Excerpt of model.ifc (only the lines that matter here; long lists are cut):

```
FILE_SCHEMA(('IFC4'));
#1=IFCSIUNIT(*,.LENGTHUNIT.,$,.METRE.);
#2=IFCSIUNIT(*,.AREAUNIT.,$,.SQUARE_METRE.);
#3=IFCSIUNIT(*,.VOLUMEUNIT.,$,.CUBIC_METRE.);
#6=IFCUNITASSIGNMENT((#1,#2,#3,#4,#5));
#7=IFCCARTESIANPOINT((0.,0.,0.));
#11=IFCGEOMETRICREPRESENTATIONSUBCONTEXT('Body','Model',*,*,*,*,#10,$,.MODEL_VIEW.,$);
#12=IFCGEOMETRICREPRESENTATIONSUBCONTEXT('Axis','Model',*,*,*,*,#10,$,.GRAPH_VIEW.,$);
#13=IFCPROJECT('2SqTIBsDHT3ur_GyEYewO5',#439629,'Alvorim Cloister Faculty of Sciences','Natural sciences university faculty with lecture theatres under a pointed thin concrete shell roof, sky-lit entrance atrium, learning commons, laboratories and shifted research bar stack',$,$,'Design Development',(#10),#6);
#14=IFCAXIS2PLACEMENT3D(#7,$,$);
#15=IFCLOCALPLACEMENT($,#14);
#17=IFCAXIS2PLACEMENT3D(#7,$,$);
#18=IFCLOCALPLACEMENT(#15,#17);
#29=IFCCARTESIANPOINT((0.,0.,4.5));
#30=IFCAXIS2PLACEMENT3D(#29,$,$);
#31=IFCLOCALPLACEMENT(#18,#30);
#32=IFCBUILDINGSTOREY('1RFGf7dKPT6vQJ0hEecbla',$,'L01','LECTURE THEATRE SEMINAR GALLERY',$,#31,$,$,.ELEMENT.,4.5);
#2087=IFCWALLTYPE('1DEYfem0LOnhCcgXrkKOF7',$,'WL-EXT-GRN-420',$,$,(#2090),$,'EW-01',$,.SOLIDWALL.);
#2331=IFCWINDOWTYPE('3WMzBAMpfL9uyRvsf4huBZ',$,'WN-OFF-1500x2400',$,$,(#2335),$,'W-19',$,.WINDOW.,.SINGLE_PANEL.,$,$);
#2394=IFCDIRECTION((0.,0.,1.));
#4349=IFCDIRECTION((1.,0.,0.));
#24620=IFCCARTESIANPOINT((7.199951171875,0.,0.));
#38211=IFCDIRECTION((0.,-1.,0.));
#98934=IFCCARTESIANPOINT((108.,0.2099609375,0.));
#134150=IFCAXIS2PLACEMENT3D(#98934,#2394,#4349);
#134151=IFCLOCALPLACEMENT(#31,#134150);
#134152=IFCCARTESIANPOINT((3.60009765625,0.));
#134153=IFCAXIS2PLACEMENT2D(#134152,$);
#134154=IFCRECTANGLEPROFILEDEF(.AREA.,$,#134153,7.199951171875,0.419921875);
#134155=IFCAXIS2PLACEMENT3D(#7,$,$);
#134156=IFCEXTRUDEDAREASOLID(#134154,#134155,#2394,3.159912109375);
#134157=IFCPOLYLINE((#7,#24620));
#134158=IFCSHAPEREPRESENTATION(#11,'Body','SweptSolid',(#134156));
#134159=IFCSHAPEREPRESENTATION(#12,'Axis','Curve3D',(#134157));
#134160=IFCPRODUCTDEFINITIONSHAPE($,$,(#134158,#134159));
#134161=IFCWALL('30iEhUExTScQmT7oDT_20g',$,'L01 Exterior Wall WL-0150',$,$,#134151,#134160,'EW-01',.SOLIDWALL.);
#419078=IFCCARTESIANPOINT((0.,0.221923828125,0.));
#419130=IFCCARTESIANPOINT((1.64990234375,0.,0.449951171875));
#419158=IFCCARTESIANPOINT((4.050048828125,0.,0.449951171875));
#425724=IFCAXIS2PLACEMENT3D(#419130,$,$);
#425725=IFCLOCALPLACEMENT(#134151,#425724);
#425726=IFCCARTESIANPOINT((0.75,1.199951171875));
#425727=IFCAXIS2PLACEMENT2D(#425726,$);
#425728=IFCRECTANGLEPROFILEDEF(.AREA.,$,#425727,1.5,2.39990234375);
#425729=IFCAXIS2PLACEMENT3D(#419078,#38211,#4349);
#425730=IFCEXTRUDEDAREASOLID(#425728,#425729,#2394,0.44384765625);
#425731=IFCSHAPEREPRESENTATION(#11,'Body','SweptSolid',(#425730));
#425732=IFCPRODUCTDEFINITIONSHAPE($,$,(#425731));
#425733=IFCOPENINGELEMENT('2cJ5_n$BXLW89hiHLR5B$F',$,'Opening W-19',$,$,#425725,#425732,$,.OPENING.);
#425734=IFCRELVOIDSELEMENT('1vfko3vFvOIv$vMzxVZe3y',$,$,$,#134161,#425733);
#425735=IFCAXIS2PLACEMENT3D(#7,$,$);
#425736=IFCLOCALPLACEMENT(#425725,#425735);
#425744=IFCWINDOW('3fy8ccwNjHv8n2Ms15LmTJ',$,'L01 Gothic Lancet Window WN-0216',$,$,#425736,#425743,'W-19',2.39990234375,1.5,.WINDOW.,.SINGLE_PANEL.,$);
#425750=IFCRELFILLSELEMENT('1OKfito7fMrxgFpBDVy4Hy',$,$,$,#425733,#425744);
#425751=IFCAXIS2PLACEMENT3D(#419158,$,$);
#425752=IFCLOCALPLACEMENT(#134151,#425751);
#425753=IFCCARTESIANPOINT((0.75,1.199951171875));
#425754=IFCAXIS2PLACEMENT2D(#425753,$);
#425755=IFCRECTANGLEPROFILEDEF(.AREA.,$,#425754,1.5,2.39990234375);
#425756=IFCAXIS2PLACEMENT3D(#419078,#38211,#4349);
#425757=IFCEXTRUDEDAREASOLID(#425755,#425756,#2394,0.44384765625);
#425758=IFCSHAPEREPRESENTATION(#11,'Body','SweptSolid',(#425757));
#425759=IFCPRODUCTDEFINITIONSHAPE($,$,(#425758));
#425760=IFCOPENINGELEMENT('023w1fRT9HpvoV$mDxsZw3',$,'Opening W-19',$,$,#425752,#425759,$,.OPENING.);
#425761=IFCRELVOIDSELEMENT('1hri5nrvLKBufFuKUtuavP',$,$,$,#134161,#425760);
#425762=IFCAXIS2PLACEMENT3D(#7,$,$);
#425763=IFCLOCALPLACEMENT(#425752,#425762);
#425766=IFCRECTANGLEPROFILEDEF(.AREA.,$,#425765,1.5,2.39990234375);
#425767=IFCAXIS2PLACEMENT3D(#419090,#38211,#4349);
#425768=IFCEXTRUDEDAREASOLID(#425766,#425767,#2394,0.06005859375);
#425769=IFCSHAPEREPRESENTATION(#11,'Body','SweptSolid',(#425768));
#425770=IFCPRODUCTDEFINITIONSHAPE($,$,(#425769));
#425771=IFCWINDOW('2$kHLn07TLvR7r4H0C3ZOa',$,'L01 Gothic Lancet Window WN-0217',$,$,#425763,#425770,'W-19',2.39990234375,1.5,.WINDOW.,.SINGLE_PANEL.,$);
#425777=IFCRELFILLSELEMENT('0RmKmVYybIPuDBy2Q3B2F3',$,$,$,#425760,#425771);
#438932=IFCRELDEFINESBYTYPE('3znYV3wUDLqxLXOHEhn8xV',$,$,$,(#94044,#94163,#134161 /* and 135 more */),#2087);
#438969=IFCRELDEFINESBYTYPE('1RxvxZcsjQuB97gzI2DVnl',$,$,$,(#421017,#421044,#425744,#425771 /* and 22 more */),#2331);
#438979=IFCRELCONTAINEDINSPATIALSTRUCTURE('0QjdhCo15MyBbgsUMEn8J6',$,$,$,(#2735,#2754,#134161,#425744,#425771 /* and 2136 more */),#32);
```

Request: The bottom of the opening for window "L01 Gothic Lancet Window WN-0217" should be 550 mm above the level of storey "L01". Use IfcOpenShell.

```python
import numpy as np
import ifcopenshell
import ifcopenshell.api.geometry
import ifcopenshell.geom
import ifcopenshell.util.element
import ifcopenshell.util.placement
import ifcopenshell.util.shape
import ifcopenshell.util.unit

model = ifcopenshell.open("model.ifc")
unit_scale = ifcopenshell.util.unit.calculate_unit_scale(model)

window = model.by_id(425771)
opening = window.FillsVoids[0].RelatingOpeningElement
storey = ifcopenshell.util.element.get_container(window, ifc_class="IfcBuildingStorey")
level = ifcopenshell.util.placement.get_local_placement(storey.ObjectPlacement)[2, 3]

# The opening's origin need not be at the sill, so measure its lowest point.
shape = ifcopenshell.geom.create_shape(ifcopenshell.geom.settings(), opening)
bottom = ifcopenshell.util.shape.get_shape_bottom_elevation(shape, shape.geometry) / unit_scale
dz = level + 0.55 / unit_scale - bottom

shift = np.array([0.0, 0.0, dz])
# The window is placed relative to its opening, so it follows when the opening moves.
matrix = ifcopenshell.util.placement.get_local_placement(opening.ObjectPlacement)
matrix[:3, 3] += shift
ifcopenshell.api.geometry.edit_object_placement(
    model, product=opening, matrix=matrix, is_si=False, should_transform_children=True
)

print(f"moved by {dz * unit_scale:+.3f} m")

model.write("model_v2.ifc")
```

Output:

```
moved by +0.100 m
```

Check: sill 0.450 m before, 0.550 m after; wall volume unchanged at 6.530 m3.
